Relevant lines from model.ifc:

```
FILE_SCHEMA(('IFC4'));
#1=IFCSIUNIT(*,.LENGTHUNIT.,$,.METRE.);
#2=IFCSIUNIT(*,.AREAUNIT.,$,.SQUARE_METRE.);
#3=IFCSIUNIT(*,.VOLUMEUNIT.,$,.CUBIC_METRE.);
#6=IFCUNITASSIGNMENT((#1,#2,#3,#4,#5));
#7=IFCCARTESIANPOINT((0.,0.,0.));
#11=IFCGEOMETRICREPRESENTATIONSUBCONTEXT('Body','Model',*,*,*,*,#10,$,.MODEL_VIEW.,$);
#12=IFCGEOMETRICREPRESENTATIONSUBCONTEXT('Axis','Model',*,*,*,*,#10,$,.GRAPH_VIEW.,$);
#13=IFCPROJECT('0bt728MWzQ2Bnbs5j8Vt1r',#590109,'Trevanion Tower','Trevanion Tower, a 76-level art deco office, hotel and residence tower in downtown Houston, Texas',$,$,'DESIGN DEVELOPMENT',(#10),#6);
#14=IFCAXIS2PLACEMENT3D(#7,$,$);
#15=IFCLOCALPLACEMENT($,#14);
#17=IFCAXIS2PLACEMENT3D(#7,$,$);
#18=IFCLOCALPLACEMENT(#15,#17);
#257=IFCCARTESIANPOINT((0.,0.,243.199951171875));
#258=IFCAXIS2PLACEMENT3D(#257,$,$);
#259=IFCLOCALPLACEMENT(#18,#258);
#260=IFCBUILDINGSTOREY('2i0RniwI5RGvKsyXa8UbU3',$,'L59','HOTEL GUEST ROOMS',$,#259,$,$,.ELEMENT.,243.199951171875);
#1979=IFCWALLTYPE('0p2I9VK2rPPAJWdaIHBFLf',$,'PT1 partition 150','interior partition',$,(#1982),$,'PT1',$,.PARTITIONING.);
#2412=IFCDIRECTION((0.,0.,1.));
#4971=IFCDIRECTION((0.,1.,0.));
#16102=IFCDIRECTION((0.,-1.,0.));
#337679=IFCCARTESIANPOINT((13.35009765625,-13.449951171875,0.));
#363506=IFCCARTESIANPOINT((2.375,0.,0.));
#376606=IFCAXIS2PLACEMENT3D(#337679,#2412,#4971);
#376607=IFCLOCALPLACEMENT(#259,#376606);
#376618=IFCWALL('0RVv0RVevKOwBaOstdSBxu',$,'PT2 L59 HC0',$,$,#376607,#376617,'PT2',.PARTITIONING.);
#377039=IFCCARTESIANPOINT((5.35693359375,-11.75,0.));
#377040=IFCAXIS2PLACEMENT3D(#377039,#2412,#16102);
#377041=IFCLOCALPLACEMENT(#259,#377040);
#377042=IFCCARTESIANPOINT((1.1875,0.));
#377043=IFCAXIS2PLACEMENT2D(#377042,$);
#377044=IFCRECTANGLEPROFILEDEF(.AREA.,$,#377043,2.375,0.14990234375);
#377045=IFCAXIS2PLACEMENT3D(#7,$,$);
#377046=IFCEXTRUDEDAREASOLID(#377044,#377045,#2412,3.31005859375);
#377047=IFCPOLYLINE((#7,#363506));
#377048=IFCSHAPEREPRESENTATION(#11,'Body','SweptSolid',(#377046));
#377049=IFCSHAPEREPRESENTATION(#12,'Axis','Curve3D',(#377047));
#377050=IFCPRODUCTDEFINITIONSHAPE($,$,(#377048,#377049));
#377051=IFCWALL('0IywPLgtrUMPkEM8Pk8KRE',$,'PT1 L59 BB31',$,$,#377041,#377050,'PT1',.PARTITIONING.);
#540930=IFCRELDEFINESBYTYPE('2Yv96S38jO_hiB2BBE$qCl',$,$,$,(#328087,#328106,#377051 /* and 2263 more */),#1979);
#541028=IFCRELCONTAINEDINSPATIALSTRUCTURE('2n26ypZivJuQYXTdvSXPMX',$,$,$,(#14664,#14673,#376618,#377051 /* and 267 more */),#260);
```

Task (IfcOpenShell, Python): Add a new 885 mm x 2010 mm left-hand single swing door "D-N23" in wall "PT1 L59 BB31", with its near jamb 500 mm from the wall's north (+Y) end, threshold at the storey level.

```python
import numpy as np
import ifcopenshell
import ifcopenshell.api.feature
import ifcopenshell.api.geometry
import ifcopenshell.api.root
import ifcopenshell.api.spatial
import ifcopenshell.geom
import ifcopenshell.util.element
import ifcopenshell.util.placement
import ifcopenshell.util.representation
import ifcopenshell.util.shape
import ifcopenshell.util.unit

model = ifcopenshell.open("model.ifc")
unit_scale = ifcopenshell.util.unit.calculate_unit_scale(model)
settings = ifcopenshell.geom.settings()


def volume(element):
    """Net volume in cubic metres, openings subtracted."""
    shape = ifcopenshell.geom.create_shape(settings, element)
    return ifcopenshell.util.shape.get_volume(shape.geometry)


wall = model.by_guid("0IywPLgtrUMPkEM8Pk8KRE")
storey = ifcopenshell.util.element.get_container(wall, ifc_class="IfcBuildingStorey")
context = ifcopenshell.util.representation.get_context(model, "Model", "Body", "MODEL_VIEW")
before = volume(wall)

width, height, from_end, sill = 0.885, 2.01, 0.5, 0.0  # metres

# The wall runs along its own X axis, and the end named is its -X end.
wall_shape = ifcopenshell.geom.create_shape(settings, wall)
x, y, z = ifcopenshell.util.shape.get_vertices(wall_shape.geometry).T
start = x.min() + from_end
face, thickness = float(y.min()), float(y.max() - y.min())
wall_matrix = ifcopenshell.util.placement.get_local_placement(wall.ObjectPlacement)
level = ifcopenshell.util.placement.get_local_placement(storey.ObjectPlacement)[2, 3]


def in_wall(x, y):
    """Placement at x, y metres in the wall's axes, at sill height."""
    matrix = wall_matrix.copy()
    matrix[:, 3] = wall_matrix @ np.array([x / unit_scale, y / unit_scale, 0.0, 1.0])
    matrix[2, 3] = level + sill / unit_scale
    return matrix


# Opening: a box that overshoots both wall faces by 50 mm.
opening = ifcopenshell.api.root.create_entity(model, ifc_class="IfcOpeningElement", predefined_type="OPENING")
box = ifcopenshell.api.geometry.add_wall_representation(
    model, context=context, length=width, height=height, thickness=thickness + 0.1
)
ifcopenshell.api.geometry.assign_representation(model, product=opening, representation=box)
ifcopenshell.api.geometry.edit_object_placement(model, product=opening, matrix=in_wall(start, face - 0.05), is_si=False)
ifcopenshell.api.feature.add_feature(model, feature=opening, element=wall)

door = ifcopenshell.api.root.create_entity(model, ifc_class="IfcDoor", name="D-N23", predefined_type="DOOR")
door.OverallWidth, door.OverallHeight = width / unit_scale, height / unit_scale
door.OperationType = "SINGLE_SWING_LEFT"
body = ifcopenshell.api.geometry.add_door_representation(
    model,
    context=context,
    overall_width=door.OverallWidth,
    overall_height=door.OverallHeight,
    operation_type="SINGLE_SWING_LEFT",
    lining_properties={"LiningDepth": thickness / unit_scale, "ThresholdDepth": thickness / unit_scale},
)
ifcopenshell.api.geometry.assign_representation(model, product=door, representation=body)
ifcopenshell.api.spatial.assign_container(model, products=[door], relating_structure=storey)
ifcopenshell.api.feature.add_filling(model, opening=opening, element=door)

# The lining spans the wall, so the door starts at the wall face.
ifcopenshell.api.geometry.edit_object_placement(model, product=door, matrix=in_wall(start, face), is_si=False)

after = volume(wall)

print(f"wall volume {before:.3f} -> {after:.3f} m3")

model.write("model_rev.ifc")
```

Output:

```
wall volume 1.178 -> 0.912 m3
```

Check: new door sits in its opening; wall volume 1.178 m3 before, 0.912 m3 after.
